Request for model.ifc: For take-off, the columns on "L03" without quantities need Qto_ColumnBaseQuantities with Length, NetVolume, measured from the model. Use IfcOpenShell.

First a look at what the model holds.

```python
import ifcopenshell
import ifcopenshell.util.element
import ifcopenshell.util.unit

model = ifcopenshell.open("model.ifc")
print(model.schema)
for unit_type in ("LENGTHUNIT", "AREAUNIT", "VOLUMEUNIT"):
    print(unit_type, ifcopenshell.util.unit.calculate_unit_scale(model, unit_type))
storey = next(s for s in model.by_type("IfcBuildingStorey") if s.Name == "L03")
columns = [e for e in ifcopenshell.util.element.get_decomposition(storey) if e.is_a("IfcColumn")]
for e in sorted(columns, key=lambda e: e.id()):
    print(e.id(), e.is_a(), e.Name, list(ifcopenshell.util.element.get_psets(e, qtos_only=True)), sep=" | ")
```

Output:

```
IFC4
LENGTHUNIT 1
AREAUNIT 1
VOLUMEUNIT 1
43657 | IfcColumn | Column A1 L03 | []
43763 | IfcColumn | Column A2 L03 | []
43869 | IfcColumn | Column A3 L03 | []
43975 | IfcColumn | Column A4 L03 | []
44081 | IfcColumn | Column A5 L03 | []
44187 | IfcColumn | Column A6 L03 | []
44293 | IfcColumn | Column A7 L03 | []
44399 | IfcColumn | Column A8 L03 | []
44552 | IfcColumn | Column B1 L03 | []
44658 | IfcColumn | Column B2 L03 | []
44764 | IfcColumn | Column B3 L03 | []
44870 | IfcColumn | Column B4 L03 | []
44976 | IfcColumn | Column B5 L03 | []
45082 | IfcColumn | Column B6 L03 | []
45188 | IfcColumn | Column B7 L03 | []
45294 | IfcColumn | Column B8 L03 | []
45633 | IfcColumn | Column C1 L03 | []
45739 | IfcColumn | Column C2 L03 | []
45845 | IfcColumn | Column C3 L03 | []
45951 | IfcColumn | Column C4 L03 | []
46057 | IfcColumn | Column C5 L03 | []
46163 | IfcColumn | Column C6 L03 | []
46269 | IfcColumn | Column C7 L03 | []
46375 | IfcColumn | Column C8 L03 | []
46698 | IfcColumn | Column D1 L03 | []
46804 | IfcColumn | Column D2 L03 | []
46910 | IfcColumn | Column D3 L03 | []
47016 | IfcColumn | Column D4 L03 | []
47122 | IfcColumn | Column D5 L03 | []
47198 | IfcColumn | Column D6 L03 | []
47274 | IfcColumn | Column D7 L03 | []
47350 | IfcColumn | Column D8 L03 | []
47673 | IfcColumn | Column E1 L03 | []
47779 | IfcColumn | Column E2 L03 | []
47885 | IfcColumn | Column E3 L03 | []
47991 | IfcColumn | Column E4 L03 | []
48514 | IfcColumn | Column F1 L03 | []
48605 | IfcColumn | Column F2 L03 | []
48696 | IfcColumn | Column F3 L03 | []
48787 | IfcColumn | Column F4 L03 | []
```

```python
import ifcopenshell
import ifcopenshell.api.pset
import ifcopenshell.geom
import ifcopenshell.util.element
import ifcopenshell.util.shape
import ifcopenshell.util.unit

model = ifcopenshell.open("model.ifc")
unit_scale = ifcopenshell.util.unit.calculate_unit_scale(model)
volume_scale = ifcopenshell.util.unit.calculate_unit_scale(model, "VOLUMEUNIT")
settings = ifcopenshell.geom.settings()

storey = next(s for s in model.by_type("IfcBuildingStorey") if s.Name == "L03")
columns = [e for e in ifcopenshell.util.element.get_decomposition(storey) if e.is_a("IfcColumn")]

for e in sorted(columns, key=lambda e: e.id()):
    if ifcopenshell.util.element.get_psets(e, qtos_only=True, should_inherit=False):
        continue
    # Geometry comes back in metres, in the element's own axes.
    shape = ifcopenshell.geom.create_shape(settings, e)
    values = {
        "Length": ifcopenshell.util.shape.get_z(shape.geometry) / unit_scale,
        "NetVolume": ifcopenshell.util.shape.get_volume(shape.geometry) / volume_scale,
    }
    qto = ifcopenshell.api.pset.add_qto(model, product=e, name="Qto_ColumnBaseQuantities")
    ifcopenshell.api.pset.edit_qto(model, qto=qto, properties=values)
    print(e.id(), {k: round(v, 3) for k, v in values.items()})

model.write("model_updated.ifc")
```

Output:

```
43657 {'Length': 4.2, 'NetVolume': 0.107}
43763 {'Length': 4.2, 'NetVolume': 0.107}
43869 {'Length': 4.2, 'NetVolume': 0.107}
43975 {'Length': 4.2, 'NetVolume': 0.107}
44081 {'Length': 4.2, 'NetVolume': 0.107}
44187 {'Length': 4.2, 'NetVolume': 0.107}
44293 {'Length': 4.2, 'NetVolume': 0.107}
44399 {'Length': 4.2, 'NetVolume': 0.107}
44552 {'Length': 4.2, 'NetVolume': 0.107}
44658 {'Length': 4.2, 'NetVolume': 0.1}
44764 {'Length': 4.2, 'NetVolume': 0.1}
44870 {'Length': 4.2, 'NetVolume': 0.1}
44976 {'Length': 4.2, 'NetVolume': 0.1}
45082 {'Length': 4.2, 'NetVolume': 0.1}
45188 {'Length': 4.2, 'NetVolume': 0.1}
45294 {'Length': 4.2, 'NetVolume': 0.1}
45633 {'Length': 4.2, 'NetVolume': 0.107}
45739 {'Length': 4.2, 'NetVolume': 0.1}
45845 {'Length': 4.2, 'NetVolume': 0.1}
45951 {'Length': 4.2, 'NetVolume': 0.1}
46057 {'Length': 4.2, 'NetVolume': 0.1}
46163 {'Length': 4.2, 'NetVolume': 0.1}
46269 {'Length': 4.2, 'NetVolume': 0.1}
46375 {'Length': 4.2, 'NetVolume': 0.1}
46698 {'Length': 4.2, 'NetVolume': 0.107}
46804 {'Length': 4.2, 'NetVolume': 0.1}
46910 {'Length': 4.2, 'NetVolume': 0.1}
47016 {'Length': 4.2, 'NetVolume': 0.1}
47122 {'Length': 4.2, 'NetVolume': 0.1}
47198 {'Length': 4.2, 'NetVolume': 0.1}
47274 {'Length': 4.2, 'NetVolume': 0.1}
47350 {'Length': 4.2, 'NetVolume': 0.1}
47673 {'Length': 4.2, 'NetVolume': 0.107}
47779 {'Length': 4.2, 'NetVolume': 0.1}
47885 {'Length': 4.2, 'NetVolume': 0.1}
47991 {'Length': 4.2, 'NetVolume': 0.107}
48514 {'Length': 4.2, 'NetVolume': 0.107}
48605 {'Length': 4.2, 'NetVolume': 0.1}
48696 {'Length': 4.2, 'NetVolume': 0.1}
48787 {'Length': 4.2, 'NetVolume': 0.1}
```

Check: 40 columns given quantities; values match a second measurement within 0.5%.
